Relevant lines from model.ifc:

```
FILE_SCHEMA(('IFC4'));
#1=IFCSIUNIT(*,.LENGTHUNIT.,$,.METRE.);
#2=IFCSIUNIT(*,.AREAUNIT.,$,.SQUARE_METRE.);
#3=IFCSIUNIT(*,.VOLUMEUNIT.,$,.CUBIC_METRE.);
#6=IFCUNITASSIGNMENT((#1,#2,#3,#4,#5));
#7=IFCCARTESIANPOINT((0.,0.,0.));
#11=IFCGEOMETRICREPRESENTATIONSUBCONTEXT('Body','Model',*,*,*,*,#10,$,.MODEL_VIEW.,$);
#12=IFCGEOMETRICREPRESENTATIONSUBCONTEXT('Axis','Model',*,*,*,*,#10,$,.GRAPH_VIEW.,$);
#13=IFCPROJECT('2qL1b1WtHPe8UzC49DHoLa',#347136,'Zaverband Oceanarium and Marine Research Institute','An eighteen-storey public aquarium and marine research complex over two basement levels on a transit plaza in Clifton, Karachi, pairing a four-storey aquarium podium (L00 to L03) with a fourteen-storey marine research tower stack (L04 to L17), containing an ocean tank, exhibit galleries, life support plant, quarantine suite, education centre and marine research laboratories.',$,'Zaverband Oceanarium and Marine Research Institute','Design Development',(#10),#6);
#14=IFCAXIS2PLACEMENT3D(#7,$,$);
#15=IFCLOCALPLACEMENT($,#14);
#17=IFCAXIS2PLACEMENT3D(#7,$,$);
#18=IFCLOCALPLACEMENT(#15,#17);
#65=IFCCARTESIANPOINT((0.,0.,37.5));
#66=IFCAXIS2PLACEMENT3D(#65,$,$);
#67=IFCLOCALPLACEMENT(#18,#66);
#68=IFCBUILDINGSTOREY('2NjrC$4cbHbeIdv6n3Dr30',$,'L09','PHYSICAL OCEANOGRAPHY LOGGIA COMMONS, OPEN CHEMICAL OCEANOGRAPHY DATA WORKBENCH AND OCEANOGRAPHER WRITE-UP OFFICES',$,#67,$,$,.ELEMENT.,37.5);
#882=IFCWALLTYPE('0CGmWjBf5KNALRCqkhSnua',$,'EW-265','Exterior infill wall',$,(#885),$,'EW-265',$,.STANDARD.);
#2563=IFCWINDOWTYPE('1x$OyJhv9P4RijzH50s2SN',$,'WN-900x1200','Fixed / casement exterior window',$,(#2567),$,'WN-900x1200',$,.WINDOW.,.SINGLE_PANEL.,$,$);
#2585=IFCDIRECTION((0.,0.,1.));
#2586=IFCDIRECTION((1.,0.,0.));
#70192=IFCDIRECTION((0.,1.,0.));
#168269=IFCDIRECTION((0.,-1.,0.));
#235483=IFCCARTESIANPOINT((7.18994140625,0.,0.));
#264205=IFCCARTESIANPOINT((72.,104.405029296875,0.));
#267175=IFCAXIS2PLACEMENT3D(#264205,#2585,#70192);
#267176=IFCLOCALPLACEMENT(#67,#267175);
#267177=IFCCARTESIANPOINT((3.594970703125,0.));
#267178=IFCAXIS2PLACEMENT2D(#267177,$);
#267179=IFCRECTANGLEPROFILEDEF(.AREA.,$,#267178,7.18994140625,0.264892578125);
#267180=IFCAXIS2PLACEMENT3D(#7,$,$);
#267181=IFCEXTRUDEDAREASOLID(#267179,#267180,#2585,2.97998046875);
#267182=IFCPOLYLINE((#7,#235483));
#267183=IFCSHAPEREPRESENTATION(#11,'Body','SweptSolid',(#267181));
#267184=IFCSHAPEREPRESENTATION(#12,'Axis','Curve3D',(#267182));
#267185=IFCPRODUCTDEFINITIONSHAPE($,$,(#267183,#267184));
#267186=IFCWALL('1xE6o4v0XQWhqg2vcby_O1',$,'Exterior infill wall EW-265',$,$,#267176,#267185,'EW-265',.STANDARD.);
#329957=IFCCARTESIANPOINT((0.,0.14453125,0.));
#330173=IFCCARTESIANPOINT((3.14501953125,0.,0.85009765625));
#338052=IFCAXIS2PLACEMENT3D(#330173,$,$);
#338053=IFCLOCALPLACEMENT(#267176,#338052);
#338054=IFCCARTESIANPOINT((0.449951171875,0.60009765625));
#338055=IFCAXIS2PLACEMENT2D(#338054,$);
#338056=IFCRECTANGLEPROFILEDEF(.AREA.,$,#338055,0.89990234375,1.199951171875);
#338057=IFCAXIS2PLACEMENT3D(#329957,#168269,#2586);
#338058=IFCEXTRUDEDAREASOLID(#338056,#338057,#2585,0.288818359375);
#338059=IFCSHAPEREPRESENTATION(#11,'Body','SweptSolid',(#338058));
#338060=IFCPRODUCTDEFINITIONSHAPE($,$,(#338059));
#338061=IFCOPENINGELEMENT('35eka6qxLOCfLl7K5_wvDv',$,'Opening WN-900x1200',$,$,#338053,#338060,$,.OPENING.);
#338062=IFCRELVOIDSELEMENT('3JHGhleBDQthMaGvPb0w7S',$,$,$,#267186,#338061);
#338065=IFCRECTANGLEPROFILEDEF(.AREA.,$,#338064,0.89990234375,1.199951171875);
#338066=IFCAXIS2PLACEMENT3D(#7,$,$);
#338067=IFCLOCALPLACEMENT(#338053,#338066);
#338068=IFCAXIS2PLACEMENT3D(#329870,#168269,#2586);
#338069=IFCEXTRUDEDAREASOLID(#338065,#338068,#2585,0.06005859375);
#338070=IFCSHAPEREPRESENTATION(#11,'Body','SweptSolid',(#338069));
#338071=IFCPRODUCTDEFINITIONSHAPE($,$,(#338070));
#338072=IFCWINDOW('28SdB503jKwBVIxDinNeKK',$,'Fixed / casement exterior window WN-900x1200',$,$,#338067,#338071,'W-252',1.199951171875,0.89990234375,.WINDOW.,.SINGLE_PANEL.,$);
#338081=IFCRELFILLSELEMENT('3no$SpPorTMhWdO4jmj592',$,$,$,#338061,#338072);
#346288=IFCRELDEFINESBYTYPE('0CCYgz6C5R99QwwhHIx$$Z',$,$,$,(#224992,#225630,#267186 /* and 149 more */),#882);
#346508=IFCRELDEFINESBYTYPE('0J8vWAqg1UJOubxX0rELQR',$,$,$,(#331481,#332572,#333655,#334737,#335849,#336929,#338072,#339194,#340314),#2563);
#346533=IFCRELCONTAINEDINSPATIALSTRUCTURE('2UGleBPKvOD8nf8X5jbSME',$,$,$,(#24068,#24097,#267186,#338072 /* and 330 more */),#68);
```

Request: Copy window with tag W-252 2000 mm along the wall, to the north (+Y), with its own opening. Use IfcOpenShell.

```python
import ifcopenshell
import ifcopenshell.api.feature
import ifcopenshell.api.geometry
import ifcopenshell.api.root
import ifcopenshell.geom
import ifcopenshell.util.element
import ifcopenshell.util.placement
import ifcopenshell.util.shape
import ifcopenshell.util.unit

model = ifcopenshell.open("model.ifc")
unit_scale = ifcopenshell.util.unit.calculate_unit_scale(model)
settings = ifcopenshell.geom.settings()


def volume(element):
    """Net volume in cubic metres, openings subtracted."""
    shape = ifcopenshell.geom.create_shape(settings, element)
    return ifcopenshell.util.shape.get_volume(shape.geometry)


window = model.by_guid("28SdB503jKwBVIxDinNeKK")
opening = window.FillsVoids[0].RelatingOpeningElement
wall = opening.VoidsElements[0].RelatingBuildingElement
before = volume(wall)
shift = ifcopenshell.util.placement.get_local_placement(wall.ObjectPlacement)[:3, 0] * 2 / unit_scale

# copy_class copies the void relationship, type, container and properties, but no geometry.
new_opening = ifcopenshell.api.root.copy_class(model, product=opening)
new_opening.Representation = ifcopenshell.util.element.copy_deep(
    model, opening.Representation, exclude=["IfcGeometricRepresentationContext", "IfcRepresentationMap"]
)
new_window = ifcopenshell.api.root.copy_class(model, product=window)
new_window.Representation = ifcopenshell.util.element.copy_deep(
    model, window.Representation, exclude=["IfcGeometricRepresentationContext", "IfcRepresentationMap"]
)
new_window.Tag = None
ifcopenshell.api.feature.add_filling(model, opening=new_opening, element=new_window)

for old, new in ((opening, new_opening), (window, new_window)):
    matrix = ifcopenshell.util.placement.get_local_placement(old.ObjectPlacement)
    matrix[:3, 3] += shift
    ifcopenshell.api.geometry.edit_object_placement(model, product=new, matrix=matrix, is_si=False)

after = volume(wall)

print(f"wall volume {before:.3f} -> {after:.3f} m3")

model.write("model_v2.ifc")
```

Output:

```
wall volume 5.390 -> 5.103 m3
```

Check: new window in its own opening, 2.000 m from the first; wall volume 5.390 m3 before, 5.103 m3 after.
